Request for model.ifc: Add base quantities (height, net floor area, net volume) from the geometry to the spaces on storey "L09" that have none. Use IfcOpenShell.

First a look at what the model holds.

```python
import ifcopenshell
import ifcopenshell.util.element
import ifcopenshell.util.unit

model = ifcopenshell.open("model.ifc")
print(model.schema)
for unit_type in ("LENGTHUNIT", "AREAUNIT", "VOLUMEUNIT"):
    print(unit_type, ifcopenshell.util.unit.calculate_unit_scale(model, unit_type))
storey = next(s for s in model.by_type("IfcBuildingStorey") if s.Name == "L09")
spaces = [e for e in ifcopenshell.util.element.get_decomposition(storey) if e.is_a("IfcSpace")]
for e in sorted(spaces, key=lambda e: e.id()):
    print(e.id(), e.is_a(), e.Name, list(ifcopenshell.util.element.get_psets(e, qtos_only=True)), sep=" | ")
```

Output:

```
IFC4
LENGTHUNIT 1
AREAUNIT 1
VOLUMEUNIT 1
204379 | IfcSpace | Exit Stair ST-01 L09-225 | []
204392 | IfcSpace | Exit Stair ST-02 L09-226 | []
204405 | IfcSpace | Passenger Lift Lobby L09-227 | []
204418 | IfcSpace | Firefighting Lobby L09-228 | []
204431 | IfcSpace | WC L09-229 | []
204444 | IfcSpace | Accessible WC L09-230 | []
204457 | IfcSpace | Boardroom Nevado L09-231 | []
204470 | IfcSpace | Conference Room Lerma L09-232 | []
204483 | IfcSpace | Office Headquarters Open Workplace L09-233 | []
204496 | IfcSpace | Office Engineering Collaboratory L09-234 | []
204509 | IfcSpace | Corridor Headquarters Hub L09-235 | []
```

```python
import ifcopenshell
import ifcopenshell.api.pset
import ifcopenshell.geom
import ifcopenshell.util.element
import ifcopenshell.util.shape
import ifcopenshell.util.unit

model = ifcopenshell.open("model.ifc")
unit_scale = ifcopenshell.util.unit.calculate_unit_scale(model)
area_scale = ifcopenshell.util.unit.calculate_unit_scale(model, "AREAUNIT")
volume_scale = ifcopenshell.util.unit.calculate_unit_scale(model, "VOLUMEUNIT")
settings = ifcopenshell.geom.settings()

storey = next(s for s in model.by_type("IfcBuildingStorey") if s.Name == "L09")
spaces = [e for e in ifcopenshell.util.element.get_decomposition(storey) if e.is_a("IfcSpace")]

for e in sorted(spaces, key=lambda e: e.id()):
    if ifcopenshell.util.element.get_psets(e, qtos_only=True, should_inherit=False):
        continue
    # Geometry comes back in metres, in the element's own axes.
    shape = ifcopenshell.geom.create_shape(settings, e)
    values = {
        "Height": ifcopenshell.util.shape.get_z(shape.geometry) / unit_scale,
        "NetFloorArea": ifcopenshell.util.shape.get_footprint_area(shape.geometry) / area_scale,
        "NetVolume": ifcopenshell.util.shape.get_volume(shape.geometry) / volume_scale,
    }
    qto = ifcopenshell.api.pset.add_qto(model, product=e, name="Qto_SpaceBaseQuantities")
    ifcopenshell.api.pset.edit_qto(model, qto=qto, properties=values)
    print(e.id(), {k: round(v, 3) for k, v in values.items()})

model.write("model_edited.ifc")
```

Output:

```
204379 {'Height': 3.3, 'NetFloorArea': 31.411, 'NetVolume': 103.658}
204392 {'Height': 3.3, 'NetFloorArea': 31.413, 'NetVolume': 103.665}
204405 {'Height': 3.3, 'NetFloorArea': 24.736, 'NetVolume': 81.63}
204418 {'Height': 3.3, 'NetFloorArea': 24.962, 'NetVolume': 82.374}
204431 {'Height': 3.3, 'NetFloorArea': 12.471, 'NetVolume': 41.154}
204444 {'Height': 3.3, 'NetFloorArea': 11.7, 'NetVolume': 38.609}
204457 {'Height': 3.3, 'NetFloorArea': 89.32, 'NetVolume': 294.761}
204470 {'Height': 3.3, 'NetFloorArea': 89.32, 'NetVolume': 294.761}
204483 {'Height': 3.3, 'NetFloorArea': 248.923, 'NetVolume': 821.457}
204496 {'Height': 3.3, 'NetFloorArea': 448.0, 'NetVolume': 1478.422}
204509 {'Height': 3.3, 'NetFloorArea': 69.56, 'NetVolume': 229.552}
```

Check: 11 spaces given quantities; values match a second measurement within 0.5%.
